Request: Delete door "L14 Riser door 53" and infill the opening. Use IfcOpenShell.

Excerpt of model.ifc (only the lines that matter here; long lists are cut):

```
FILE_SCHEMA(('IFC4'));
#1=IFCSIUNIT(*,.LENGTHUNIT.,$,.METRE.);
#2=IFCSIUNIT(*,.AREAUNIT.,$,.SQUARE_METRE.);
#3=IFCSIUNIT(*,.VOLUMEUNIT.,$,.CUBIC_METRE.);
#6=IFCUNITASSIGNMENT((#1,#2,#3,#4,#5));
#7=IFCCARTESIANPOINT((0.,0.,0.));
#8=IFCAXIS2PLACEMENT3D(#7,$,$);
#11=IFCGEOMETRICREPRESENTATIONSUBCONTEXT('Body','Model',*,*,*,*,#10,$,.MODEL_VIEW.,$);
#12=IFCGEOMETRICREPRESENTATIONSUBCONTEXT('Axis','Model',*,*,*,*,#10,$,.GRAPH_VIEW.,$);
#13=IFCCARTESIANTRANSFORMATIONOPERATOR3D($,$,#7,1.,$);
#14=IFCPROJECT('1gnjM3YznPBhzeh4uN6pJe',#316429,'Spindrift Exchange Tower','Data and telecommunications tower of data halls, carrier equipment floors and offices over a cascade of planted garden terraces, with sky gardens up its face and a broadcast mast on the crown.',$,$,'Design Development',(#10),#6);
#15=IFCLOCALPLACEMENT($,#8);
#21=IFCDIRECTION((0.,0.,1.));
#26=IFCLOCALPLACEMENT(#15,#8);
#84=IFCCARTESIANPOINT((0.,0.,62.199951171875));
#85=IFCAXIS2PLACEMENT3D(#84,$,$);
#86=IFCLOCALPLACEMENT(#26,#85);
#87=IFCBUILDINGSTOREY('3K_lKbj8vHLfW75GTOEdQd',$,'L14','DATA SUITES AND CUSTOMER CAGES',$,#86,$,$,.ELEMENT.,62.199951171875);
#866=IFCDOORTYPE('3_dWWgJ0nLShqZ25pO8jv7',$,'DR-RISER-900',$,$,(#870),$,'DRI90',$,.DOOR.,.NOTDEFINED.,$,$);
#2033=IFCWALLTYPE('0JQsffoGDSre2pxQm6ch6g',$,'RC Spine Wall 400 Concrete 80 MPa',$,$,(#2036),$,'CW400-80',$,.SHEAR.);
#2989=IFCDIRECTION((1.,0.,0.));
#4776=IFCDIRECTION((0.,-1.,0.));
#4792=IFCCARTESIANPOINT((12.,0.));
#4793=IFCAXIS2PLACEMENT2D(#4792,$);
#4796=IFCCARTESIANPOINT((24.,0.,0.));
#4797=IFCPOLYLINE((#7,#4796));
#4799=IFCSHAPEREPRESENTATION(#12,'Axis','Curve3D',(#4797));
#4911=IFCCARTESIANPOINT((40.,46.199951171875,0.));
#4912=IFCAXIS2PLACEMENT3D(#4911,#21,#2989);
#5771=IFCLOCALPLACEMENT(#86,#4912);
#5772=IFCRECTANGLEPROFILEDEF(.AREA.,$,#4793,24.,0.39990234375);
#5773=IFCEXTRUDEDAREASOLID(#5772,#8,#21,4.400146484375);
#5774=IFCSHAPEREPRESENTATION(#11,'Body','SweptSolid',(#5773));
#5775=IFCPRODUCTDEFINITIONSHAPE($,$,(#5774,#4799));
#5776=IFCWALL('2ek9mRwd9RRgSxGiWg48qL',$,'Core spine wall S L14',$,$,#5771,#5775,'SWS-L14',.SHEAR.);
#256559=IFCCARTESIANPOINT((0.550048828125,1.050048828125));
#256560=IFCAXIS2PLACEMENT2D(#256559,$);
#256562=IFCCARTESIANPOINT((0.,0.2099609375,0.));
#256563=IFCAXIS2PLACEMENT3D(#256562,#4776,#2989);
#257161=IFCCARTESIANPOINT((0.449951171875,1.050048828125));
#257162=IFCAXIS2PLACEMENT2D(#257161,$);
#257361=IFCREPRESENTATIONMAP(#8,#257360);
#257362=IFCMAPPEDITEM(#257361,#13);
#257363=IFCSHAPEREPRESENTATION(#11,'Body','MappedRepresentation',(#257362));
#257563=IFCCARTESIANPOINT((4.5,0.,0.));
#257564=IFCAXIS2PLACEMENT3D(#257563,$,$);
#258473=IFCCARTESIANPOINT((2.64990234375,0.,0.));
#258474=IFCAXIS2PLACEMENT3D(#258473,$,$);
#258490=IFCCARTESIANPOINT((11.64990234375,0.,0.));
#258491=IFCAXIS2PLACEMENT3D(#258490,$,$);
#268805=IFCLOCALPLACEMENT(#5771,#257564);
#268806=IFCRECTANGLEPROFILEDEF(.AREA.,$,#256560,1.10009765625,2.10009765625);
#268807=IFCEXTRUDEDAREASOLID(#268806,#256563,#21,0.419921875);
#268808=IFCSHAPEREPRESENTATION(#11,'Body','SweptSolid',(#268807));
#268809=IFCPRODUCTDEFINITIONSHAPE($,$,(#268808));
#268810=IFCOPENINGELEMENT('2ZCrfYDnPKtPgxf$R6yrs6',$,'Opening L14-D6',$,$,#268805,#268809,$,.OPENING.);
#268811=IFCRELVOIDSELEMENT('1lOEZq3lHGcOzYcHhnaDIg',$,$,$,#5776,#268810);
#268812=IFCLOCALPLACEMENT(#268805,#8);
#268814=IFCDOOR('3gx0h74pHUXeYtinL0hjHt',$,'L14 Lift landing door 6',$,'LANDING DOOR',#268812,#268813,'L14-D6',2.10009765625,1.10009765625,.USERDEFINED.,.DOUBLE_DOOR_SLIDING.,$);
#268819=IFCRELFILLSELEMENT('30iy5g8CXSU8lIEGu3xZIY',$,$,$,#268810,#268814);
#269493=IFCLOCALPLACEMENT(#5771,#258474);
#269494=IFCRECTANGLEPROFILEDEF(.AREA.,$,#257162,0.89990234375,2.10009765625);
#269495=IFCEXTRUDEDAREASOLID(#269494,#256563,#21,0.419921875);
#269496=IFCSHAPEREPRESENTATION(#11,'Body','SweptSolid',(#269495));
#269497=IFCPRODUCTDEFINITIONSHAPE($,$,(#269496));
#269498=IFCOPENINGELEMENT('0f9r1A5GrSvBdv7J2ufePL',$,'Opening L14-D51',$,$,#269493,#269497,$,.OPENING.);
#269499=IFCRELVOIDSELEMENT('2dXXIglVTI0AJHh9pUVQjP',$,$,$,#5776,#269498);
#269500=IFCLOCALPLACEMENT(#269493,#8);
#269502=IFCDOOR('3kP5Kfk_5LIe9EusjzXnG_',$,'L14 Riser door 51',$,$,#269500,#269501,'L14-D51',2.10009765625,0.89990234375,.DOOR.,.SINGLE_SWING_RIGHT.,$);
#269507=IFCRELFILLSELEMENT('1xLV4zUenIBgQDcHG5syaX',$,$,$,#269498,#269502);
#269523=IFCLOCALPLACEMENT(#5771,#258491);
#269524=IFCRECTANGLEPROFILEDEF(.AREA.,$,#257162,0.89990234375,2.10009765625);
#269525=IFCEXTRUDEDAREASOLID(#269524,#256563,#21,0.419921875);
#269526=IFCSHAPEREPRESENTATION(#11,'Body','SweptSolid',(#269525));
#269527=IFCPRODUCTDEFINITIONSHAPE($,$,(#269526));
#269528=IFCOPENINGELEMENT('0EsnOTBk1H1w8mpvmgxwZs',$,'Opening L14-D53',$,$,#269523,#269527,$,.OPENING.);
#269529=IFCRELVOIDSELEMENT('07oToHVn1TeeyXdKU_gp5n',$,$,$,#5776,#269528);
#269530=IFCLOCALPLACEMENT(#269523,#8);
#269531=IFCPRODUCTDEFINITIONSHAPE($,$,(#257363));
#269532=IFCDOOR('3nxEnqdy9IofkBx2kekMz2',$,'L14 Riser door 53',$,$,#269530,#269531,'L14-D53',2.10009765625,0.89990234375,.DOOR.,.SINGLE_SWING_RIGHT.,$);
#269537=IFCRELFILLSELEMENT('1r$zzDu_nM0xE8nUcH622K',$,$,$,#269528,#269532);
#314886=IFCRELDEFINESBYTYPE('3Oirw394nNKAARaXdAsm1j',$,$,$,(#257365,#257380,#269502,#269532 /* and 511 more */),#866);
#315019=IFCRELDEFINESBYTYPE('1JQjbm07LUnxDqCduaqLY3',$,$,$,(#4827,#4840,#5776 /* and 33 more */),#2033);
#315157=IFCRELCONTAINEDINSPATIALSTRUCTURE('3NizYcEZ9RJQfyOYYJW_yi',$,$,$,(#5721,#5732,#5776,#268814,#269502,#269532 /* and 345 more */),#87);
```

```python
import ifcopenshell
import ifcopenshell.api.feature
import ifcopenshell.api.root
import ifcopenshell.geom
import ifcopenshell.util.shape

model = ifcopenshell.open("model.ifc")
settings = ifcopenshell.geom.settings()


def volume(element):
    """Net volume in cubic metres, openings subtracted."""
    shape = ifcopenshell.geom.create_shape(settings, element)
    return ifcopenshell.util.shape.get_volume(shape.geometry)


door = model.by_id(269532)
opening = door.FillsVoids[0].RelatingOpeningElement
wall = opening.VoidsElements[0].RelatingBuildingElement
before = volume(wall)

ifcopenshell.api.root.remove_product(model, product=door)
ifcopenshell.api.feature.remove_feature(model, feature=opening)

after = volume(wall)

print(f"wall volume {before:.3f} -> {after:.3f} m3")

model.write("model-out.ifc")
```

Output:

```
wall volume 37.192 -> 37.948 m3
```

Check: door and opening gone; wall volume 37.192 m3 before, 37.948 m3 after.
